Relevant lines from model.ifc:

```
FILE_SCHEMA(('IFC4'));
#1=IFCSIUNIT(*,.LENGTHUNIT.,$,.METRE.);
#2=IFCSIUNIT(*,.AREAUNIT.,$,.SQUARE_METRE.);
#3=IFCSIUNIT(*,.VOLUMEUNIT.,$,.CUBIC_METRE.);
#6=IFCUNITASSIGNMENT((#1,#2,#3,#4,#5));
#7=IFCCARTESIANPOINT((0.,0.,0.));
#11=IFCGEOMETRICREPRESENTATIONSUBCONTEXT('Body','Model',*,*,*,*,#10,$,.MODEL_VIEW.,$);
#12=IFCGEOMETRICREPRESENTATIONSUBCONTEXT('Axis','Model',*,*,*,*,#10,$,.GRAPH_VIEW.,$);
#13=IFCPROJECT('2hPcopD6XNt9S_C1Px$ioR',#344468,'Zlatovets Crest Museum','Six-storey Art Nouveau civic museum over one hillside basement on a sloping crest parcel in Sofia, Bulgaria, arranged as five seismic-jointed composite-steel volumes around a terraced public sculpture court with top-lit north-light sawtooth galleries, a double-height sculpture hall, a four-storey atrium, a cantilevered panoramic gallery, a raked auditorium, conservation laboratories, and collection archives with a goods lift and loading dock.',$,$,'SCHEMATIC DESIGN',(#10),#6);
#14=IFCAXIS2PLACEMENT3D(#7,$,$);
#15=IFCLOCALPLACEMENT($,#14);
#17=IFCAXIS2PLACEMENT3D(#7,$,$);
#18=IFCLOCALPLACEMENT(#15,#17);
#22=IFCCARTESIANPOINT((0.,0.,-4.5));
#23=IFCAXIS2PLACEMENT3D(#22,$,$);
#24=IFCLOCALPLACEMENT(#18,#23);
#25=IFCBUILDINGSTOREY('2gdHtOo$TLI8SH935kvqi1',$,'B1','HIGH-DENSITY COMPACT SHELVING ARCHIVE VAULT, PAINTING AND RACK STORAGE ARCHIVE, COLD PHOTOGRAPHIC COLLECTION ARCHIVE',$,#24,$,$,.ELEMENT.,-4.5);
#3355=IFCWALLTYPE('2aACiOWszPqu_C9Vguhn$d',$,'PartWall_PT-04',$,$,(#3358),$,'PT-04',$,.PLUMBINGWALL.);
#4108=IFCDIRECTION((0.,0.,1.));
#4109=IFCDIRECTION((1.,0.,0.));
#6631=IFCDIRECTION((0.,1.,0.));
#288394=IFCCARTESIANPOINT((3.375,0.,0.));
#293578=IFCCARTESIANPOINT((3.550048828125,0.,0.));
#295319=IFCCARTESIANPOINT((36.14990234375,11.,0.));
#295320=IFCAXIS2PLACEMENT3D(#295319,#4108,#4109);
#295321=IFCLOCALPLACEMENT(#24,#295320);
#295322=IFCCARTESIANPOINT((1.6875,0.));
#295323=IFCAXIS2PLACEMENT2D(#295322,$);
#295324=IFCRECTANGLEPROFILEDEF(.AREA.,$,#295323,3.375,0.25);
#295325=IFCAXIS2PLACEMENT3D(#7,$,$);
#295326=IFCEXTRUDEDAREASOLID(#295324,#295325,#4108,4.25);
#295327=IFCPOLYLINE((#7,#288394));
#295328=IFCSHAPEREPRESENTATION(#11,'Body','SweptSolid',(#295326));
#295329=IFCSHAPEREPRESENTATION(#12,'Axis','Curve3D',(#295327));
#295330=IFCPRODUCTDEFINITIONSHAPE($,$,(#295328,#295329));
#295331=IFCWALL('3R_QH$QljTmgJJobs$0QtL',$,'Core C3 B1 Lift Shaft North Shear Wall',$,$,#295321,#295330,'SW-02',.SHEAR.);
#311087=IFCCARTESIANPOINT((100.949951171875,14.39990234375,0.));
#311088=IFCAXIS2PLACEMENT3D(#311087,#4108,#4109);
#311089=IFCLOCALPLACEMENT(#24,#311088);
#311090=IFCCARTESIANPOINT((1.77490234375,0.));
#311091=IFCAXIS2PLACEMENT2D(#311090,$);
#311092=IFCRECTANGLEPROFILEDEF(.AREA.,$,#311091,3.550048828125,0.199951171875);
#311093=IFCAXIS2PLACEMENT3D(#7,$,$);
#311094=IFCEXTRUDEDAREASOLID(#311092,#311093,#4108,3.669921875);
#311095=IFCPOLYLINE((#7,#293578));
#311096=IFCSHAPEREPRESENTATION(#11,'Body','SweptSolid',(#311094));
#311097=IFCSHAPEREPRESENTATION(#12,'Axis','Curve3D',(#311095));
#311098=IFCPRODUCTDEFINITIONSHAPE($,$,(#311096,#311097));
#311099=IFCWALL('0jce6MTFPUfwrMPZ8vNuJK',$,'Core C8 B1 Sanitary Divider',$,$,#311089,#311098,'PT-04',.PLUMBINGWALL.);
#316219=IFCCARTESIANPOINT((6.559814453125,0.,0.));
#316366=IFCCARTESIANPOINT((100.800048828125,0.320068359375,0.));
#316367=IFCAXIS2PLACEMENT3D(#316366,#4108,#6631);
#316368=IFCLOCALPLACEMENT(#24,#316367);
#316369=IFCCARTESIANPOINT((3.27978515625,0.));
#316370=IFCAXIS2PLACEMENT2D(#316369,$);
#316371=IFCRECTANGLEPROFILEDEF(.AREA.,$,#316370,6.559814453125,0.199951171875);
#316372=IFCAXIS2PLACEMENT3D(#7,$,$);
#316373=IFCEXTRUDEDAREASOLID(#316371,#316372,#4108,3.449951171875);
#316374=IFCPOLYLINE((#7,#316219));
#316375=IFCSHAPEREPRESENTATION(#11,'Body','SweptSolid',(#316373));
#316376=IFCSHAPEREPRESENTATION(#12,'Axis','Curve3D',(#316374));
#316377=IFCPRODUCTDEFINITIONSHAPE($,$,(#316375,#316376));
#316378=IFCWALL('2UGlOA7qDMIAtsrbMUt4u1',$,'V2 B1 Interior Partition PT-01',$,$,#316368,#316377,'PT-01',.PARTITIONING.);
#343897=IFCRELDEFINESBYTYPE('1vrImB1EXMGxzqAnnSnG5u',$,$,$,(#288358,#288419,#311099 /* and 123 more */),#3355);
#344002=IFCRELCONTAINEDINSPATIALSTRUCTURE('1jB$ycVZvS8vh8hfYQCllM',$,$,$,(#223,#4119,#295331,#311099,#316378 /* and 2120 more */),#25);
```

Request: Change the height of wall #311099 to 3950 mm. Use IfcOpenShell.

```python
import ifcopenshell
import ifcopenshell.geom
import ifcopenshell.util.representation
import ifcopenshell.util.shape
import ifcopenshell.util.unit

model = ifcopenshell.open("model.ifc")
unit_scale = ifcopenshell.util.unit.calculate_unit_scale(model)
settings = ifcopenshell.geom.settings()


def volume(element):
    """Net volume in cubic metres, openings subtracted."""
    shape = ifcopenshell.geom.create_shape(settings, element)
    return ifcopenshell.util.shape.get_volume(shape.geometry)


wall = model.by_guid("0jce6MTFPUfwrMPZ8vNuJK")
before = volume(wall)

body = ifcopenshell.util.representation.get_representation(wall, "Model", "Body")
solid = body.Items[0]
old_height = solid.Depth
solid.Depth = 3.95 / unit_scale
after = volume(wall)

print(f"height {old_height:g} -> {solid.Depth:g}, volume {before:.3f} -> {after:.3f} m3")

model.write("model_updated.ifc")
```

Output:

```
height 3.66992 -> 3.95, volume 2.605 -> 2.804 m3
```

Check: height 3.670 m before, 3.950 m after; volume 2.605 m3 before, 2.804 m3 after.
